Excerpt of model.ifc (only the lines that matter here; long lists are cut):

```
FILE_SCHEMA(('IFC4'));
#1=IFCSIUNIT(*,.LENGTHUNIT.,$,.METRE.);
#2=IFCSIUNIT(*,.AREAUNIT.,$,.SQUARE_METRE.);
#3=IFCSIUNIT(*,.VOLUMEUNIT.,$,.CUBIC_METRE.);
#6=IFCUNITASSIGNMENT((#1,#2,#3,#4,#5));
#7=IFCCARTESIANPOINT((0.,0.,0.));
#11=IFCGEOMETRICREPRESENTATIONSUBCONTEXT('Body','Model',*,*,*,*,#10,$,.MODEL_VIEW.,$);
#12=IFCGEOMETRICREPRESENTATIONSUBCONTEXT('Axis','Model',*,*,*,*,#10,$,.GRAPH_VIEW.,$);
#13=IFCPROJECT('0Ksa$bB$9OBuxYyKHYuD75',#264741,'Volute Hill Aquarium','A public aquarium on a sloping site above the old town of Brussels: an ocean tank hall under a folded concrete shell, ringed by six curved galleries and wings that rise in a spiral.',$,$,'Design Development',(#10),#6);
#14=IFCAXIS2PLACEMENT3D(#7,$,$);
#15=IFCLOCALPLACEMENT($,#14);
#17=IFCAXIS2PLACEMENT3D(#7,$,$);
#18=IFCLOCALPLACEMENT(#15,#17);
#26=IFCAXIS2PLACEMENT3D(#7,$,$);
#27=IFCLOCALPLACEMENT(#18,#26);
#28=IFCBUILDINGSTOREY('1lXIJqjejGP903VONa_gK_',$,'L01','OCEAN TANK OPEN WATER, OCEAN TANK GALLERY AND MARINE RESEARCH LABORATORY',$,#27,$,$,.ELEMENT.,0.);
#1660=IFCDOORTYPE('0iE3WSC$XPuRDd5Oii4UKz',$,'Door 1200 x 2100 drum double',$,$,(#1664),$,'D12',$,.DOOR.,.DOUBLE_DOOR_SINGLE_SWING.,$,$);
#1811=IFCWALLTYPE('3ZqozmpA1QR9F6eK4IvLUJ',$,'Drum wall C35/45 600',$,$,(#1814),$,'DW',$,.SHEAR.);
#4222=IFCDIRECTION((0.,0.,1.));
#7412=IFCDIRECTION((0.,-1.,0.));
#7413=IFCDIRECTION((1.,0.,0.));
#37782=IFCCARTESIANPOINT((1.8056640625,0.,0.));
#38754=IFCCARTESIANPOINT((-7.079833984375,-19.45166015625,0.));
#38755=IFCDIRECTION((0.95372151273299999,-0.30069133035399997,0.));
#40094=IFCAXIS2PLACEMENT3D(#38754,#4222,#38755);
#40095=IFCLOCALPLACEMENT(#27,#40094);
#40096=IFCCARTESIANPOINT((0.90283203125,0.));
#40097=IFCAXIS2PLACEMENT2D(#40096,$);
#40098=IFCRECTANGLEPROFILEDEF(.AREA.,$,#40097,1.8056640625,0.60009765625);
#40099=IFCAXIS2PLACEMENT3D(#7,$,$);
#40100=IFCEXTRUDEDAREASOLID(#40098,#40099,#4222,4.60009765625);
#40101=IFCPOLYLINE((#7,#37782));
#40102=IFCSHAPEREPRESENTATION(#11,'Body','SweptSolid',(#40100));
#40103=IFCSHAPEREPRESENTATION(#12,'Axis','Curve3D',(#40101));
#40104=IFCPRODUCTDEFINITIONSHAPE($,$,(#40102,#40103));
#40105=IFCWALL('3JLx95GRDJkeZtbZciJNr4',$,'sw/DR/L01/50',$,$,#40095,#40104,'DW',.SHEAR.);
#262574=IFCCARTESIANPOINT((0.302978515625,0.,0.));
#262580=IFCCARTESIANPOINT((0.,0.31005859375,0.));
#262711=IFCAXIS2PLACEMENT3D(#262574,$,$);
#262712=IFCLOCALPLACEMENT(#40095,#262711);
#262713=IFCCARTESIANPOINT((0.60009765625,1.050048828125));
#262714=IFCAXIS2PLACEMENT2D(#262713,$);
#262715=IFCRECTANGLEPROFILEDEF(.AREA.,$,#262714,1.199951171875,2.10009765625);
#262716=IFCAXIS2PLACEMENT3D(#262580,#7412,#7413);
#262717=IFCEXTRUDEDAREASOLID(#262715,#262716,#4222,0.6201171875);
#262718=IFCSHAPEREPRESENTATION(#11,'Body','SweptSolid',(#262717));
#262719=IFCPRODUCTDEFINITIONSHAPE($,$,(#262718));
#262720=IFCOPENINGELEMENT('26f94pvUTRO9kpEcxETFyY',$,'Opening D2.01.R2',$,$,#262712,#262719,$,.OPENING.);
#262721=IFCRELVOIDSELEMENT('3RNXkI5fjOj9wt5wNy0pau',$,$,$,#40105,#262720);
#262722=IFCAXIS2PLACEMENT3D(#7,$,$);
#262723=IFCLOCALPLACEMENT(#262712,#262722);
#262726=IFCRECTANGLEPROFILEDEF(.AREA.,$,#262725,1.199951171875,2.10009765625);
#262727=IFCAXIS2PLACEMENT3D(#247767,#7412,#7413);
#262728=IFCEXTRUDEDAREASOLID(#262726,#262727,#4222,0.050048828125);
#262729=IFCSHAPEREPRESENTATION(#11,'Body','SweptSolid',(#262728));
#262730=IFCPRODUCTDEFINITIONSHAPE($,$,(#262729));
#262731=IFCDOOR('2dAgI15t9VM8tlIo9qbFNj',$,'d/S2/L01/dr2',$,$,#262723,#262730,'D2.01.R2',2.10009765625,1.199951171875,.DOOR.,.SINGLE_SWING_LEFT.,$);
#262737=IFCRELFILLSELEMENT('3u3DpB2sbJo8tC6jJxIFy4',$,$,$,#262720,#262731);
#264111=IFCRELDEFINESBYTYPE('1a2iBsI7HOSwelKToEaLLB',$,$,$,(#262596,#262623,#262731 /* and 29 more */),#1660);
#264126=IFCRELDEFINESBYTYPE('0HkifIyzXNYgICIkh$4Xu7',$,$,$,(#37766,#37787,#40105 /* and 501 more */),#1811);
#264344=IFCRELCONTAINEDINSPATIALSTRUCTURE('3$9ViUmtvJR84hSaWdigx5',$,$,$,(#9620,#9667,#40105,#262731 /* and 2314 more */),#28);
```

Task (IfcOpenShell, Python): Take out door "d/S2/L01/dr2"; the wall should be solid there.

```python
import ifcopenshell
import ifcopenshell.api.feature
import ifcopenshell.api.root
import ifcopenshell.geom
import ifcopenshell.util.shape

model = ifcopenshell.open("model.ifc")
settings = ifcopenshell.geom.settings()


def volume(element):
    """Net volume in cubic metres, openings subtracted."""
    shape = ifcopenshell.geom.create_shape(settings, element)
    return ifcopenshell.util.shape.get_volume(shape.geometry)


door = model.by_guid("2dAgI15t9VM8tlIo9qbFNj")
opening = door.FillsVoids[0].RelatingOpeningElement
wall = opening.VoidsElements[0].RelatingBuildingElement
before = volume(wall)

ifcopenshell.api.root.remove_product(model, product=door)
ifcopenshell.api.feature.remove_feature(model, feature=opening)

after = volume(wall)

print(f"wall volume {before:.3f} -> {after:.3f} m3")

model.write("model_updated.ifc")
```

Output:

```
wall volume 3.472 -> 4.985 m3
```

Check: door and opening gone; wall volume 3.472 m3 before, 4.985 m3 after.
